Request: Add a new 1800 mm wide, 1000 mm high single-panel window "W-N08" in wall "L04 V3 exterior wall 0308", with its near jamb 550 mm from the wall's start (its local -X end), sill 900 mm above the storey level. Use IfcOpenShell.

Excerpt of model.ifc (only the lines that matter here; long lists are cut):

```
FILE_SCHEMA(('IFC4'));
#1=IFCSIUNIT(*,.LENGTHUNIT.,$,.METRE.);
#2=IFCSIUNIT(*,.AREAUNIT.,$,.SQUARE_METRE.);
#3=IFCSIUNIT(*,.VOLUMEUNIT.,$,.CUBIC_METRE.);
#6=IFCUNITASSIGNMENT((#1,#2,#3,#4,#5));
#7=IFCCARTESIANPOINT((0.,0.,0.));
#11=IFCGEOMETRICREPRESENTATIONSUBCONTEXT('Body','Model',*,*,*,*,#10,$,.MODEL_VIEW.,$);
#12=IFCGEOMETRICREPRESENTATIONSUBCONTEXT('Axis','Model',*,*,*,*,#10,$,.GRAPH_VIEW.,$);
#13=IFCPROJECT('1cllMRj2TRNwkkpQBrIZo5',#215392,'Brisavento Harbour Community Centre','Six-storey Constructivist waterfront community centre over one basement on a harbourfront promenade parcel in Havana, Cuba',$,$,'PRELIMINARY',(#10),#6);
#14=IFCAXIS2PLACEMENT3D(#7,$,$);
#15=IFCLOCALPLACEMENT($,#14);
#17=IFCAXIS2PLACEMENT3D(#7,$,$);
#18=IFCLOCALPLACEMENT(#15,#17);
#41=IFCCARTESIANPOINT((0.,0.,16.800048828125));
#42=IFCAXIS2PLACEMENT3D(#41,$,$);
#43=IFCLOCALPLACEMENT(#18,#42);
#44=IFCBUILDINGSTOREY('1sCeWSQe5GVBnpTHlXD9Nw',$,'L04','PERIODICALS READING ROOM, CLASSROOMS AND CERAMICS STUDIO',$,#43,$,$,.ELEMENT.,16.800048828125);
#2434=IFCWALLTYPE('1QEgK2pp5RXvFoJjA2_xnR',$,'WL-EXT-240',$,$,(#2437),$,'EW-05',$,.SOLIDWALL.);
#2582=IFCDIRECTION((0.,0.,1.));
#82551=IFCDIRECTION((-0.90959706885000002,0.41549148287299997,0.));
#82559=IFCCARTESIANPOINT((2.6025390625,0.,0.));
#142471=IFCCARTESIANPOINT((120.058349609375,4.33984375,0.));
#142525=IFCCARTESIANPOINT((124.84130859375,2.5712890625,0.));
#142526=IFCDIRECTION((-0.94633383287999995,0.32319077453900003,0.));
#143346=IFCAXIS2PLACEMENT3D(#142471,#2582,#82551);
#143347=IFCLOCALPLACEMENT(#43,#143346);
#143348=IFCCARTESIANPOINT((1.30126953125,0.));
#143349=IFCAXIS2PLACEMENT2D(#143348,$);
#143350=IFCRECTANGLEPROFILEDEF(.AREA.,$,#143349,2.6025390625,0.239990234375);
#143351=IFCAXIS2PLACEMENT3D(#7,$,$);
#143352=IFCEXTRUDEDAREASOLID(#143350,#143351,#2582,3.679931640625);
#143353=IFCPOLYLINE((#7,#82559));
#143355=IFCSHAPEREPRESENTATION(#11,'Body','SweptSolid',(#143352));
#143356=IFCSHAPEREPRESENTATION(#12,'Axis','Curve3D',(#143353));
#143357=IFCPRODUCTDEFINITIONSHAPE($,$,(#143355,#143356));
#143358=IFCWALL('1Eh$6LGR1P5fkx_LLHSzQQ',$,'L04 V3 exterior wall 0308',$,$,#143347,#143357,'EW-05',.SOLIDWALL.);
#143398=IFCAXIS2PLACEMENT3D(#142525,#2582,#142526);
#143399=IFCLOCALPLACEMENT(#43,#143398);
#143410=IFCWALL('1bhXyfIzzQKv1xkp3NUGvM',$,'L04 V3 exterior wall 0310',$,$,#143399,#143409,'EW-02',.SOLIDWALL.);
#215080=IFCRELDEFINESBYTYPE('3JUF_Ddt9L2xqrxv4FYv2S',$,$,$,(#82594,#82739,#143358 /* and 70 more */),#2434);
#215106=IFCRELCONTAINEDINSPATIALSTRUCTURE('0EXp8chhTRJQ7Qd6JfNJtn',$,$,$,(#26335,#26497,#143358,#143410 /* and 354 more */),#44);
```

```python
import numpy as np
import ifcopenshell
import ifcopenshell.api.feature
import ifcopenshell.api.geometry
import ifcopenshell.api.root
import ifcopenshell.api.spatial
import ifcopenshell.geom
import ifcopenshell.util.element
import ifcopenshell.util.placement
import ifcopenshell.util.representation
import ifcopenshell.util.shape
import ifcopenshell.util.unit

model = ifcopenshell.open("model.ifc")
unit_scale = ifcopenshell.util.unit.calculate_unit_scale(model)
settings = ifcopenshell.geom.settings()


def volume(element):
    """Net volume in cubic metres, openings subtracted."""
    shape = ifcopenshell.geom.create_shape(settings, element)
    return ifcopenshell.util.shape.get_volume(shape.geometry)


wall = model.by_guid("1Eh$6LGR1P5fkx_LLHSzQQ")
storey = ifcopenshell.util.element.get_container(wall, ifc_class="IfcBuildingStorey")
context = ifcopenshell.util.representation.get_context(model, "Model", "Body", "MODEL_VIEW")
before = volume(wall)

width, height, from_end, sill = 1.8, 1, 0.55, 0.9  # metres

# The wall runs along its own X axis, and the end named is its -X end.
wall_shape = ifcopenshell.geom.create_shape(settings, wall)
x, y, z = ifcopenshell.util.shape.get_vertices(wall_shape.geometry).T
start = x.min() + from_end
face, thickness = float(y.min()), float(y.max() - y.min())
wall_matrix = ifcopenshell.util.placement.get_local_placement(wall.ObjectPlacement)
level = ifcopenshell.util.placement.get_local_placement(storey.ObjectPlacement)[2, 3]


def in_wall(x, y):
    """Placement at x, y metres in the wall's axes, at sill height."""
    matrix = wall_matrix.copy()
    matrix[:, 3] = wall_matrix @ np.array([x / unit_scale, y / unit_scale, 0.0, 1.0])
    matrix[2, 3] = level + sill / unit_scale
    return matrix


# Opening: a box that overshoots both wall faces by 50 mm.
opening = ifcopenshell.api.root.create_entity(model, ifc_class="IfcOpeningElement", predefined_type="OPENING")
box = ifcopenshell.api.geometry.add_wall_representation(
    model, context=context, length=width, height=height, thickness=thickness + 0.1
)
ifcopenshell.api.geometry.assign_representation(model, product=opening, representation=box)
ifcopenshell.api.geometry.edit_object_placement(model, product=opening, matrix=in_wall(start, face - 0.05), is_si=False)
ifcopenshell.api.feature.add_feature(model, feature=opening, element=wall)

window = ifcopenshell.api.root.create_entity(model, ifc_class="IfcWindow", name="W-N08", predefined_type="WINDOW")
window.OverallWidth, window.OverallHeight = width / unit_scale, height / unit_scale
window.PartitioningType = "SINGLE_PANEL"
body = ifcopenshell.api.geometry.add_window_representation(
    model,
    context=context,
    overall_width=window.OverallWidth,
    overall_height=window.OverallHeight,
    partition_type="SINGLE_PANEL",
)
ifcopenshell.api.geometry.assign_representation(model, product=window, representation=body)
ifcopenshell.api.spatial.assign_container(model, products=[window], relating_structure=storey)
ifcopenshell.api.feature.add_filling(model, opening=opening, element=window)

# Centre the window in the wall's thickness.
ifcopenshell.api.geometry.edit_object_placement(model, product=window, matrix=in_wall(start, face), is_si=False)
window_shape = ifcopenshell.geom.create_shape(settings, window)
depth = ifcopenshell.util.shape.get_vertices(window_shape.geometry)[:, 1]
offset = face + thickness / 2 - (depth.min() + depth.max()) / 2
ifcopenshell.api.geometry.edit_object_placement(model, product=window, matrix=in_wall(start, offset), is_si=False)

after = volume(wall)

print(f"wall volume {before:.3f} -> {after:.3f} m3")

model.write("model-out.ifc")
```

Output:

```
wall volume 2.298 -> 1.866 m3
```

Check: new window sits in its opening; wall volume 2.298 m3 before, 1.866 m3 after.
